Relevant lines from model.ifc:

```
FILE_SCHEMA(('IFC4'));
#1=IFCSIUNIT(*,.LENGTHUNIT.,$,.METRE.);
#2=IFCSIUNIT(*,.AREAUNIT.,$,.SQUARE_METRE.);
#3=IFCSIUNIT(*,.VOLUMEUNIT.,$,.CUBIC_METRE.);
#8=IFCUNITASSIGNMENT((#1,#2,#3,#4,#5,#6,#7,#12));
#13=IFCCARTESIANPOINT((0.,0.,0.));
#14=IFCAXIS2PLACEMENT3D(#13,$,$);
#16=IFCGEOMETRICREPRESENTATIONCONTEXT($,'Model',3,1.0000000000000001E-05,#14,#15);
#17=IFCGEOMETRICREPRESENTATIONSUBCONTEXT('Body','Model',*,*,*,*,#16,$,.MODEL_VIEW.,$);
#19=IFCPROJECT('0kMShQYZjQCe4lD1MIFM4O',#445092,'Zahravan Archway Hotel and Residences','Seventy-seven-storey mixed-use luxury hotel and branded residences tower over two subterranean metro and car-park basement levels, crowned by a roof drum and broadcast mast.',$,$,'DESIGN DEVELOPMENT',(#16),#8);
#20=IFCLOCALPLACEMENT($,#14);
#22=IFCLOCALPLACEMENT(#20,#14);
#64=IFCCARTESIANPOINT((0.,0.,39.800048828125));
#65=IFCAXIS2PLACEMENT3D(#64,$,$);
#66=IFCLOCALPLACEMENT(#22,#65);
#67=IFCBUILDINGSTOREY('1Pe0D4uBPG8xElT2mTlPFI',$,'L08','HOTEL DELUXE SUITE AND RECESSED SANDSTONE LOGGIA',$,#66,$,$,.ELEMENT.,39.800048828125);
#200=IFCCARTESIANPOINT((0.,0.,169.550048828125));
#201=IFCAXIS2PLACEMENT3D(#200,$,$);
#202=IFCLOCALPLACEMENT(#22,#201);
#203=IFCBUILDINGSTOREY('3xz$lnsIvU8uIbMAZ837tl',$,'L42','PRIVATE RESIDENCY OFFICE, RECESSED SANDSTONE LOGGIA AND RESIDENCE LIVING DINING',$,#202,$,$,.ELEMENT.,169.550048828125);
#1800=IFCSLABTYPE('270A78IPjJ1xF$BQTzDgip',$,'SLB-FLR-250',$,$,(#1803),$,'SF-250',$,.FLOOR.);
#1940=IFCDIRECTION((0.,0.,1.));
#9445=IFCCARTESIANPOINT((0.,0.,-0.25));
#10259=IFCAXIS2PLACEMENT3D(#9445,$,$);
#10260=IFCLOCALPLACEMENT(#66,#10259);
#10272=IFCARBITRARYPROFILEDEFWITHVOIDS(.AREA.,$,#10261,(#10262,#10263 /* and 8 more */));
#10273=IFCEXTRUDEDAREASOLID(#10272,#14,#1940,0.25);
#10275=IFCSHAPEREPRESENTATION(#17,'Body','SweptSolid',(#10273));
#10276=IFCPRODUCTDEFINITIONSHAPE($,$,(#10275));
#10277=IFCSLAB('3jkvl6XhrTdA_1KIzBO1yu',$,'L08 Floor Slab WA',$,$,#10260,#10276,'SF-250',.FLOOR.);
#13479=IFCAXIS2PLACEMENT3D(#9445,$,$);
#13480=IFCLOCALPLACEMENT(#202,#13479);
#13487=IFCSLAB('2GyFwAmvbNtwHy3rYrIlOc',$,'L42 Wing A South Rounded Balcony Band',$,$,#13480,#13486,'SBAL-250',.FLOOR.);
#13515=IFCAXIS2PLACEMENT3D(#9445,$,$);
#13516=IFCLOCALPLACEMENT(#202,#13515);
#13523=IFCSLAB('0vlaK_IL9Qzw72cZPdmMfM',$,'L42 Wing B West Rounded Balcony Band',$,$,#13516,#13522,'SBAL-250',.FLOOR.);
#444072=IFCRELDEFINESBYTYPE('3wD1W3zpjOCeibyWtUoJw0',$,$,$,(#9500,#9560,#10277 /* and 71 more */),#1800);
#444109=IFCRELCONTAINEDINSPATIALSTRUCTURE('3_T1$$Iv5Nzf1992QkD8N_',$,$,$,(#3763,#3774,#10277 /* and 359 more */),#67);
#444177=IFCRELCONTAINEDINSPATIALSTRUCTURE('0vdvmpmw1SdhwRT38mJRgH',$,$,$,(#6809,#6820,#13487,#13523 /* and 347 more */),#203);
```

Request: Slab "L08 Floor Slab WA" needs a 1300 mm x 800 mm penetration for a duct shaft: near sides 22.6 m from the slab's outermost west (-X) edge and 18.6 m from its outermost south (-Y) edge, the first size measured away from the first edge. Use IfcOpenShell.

```python
import numpy as np
import ifcopenshell
import ifcopenshell.api.feature
import ifcopenshell.api.geometry
import ifcopenshell.api.root
import ifcopenshell.geom
import ifcopenshell.util.placement
import ifcopenshell.util.representation
import ifcopenshell.util.shape
import ifcopenshell.util.unit

model = ifcopenshell.open("model.ifc")
unit_scale = ifcopenshell.util.unit.calculate_unit_scale(model)
settings = ifcopenshell.geom.settings()


def volume(element):
    """Net volume in cubic metres, openings subtracted."""
    shape = ifcopenshell.geom.create_shape(settings, element)
    return ifcopenshell.util.shape.get_volume(shape.geometry)


slab = model.by_guid("3jkvl6XhrTdA_1KIzBO1yu")
before = volume(slab)

# Extent in the slab's own axes, in metres. The edges named are its -X and -Y sides.
slab_shape = ifcopenshell.geom.create_shape(settings, slab)
vertices = ifcopenshell.util.shape.get_vertices(slab_shape.geometry)
x_min, y_min, bottom = vertices.min(axis=0)
top = vertices[:, 2].max()

opening = ifcopenshell.api.root.create_entity(model, ifc_class="IfcOpeningElement", name="Duct shaft opening", predefined_type="OPENING")
context = ifcopenshell.util.representation.get_context(model, "Model", "Body", "MODEL_VIEW")
width, depth = 1.3, 0.8
outline = [(0.0, 0.0), (width, 0.0), (width, depth), (0.0, depth), (0.0, 0.0)]
# Overshoot both faces by 50 mm so the cut is clean.
shape = ifcopenshell.api.geometry.add_slab_representation(
    model, context=context, depth=top - bottom + 0.1, polyline=outline
)
ifcopenshell.api.geometry.assign_representation(model, product=opening, representation=shape)

matrix = ifcopenshell.util.placement.get_local_placement(slab.ObjectPlacement)
matrix[:, 3] = matrix @ np.append(np.array([x_min + 22.6, y_min + 18.6, bottom - 0.05]) / unit_scale, 1.0)
ifcopenshell.api.geometry.edit_object_placement(model, product=opening, matrix=matrix, is_si=False)
ifcopenshell.api.feature.add_feature(model, feature=opening, element=slab)

after = volume(slab)

print(f"slab volume {before:.3f} -> {after:.3f} m3")

model.write("model_updated.ifc")
```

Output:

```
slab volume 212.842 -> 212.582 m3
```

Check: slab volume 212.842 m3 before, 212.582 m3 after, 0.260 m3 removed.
